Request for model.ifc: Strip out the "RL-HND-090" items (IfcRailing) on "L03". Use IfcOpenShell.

First a look at what the model holds.

```python
import ifcopenshell
import ifcopenshell.util.element

model = ifcopenshell.open("model.ifc")
print(model.schema)
storey = next(s for s in model.by_type("IfcBuildingStorey") if s.Name == "L03")
railings = [e for e in ifcopenshell.util.element.get_decomposition(storey) if e.is_a("IfcRailing")]
seen = {}
for e in railings:
    element_type = ifcopenshell.util.element.get_type(e)
    name = element_type.Name if element_type not in (None, e) else None
    seen[name] = seen.get(name, 0) + 1
for name, count in sorted(seen.items(), key=str):
    print(count, "x", name)
```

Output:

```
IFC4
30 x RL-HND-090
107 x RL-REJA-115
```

```python
import ifcopenshell
import ifcopenshell.api.root
import ifcopenshell.util.element

model = ifcopenshell.open("model.ifc")

storey = next(s for s in model.by_type("IfcBuildingStorey") if s.Name == "L03")
railings = [e for e in ifcopenshell.util.element.get_decomposition(storey) if e.is_a("IfcRailing")]
targets = [e for e in railings if (t := ifcopenshell.util.element.get_type(e)) not in (None, e) and t.Name == "RL-HND-090"]

for e in targets:
    ifcopenshell.api.root.remove_product(model, product=e)
print(len(targets), "removed")

model.write("model_v2.ifc")
```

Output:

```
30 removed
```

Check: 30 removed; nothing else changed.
